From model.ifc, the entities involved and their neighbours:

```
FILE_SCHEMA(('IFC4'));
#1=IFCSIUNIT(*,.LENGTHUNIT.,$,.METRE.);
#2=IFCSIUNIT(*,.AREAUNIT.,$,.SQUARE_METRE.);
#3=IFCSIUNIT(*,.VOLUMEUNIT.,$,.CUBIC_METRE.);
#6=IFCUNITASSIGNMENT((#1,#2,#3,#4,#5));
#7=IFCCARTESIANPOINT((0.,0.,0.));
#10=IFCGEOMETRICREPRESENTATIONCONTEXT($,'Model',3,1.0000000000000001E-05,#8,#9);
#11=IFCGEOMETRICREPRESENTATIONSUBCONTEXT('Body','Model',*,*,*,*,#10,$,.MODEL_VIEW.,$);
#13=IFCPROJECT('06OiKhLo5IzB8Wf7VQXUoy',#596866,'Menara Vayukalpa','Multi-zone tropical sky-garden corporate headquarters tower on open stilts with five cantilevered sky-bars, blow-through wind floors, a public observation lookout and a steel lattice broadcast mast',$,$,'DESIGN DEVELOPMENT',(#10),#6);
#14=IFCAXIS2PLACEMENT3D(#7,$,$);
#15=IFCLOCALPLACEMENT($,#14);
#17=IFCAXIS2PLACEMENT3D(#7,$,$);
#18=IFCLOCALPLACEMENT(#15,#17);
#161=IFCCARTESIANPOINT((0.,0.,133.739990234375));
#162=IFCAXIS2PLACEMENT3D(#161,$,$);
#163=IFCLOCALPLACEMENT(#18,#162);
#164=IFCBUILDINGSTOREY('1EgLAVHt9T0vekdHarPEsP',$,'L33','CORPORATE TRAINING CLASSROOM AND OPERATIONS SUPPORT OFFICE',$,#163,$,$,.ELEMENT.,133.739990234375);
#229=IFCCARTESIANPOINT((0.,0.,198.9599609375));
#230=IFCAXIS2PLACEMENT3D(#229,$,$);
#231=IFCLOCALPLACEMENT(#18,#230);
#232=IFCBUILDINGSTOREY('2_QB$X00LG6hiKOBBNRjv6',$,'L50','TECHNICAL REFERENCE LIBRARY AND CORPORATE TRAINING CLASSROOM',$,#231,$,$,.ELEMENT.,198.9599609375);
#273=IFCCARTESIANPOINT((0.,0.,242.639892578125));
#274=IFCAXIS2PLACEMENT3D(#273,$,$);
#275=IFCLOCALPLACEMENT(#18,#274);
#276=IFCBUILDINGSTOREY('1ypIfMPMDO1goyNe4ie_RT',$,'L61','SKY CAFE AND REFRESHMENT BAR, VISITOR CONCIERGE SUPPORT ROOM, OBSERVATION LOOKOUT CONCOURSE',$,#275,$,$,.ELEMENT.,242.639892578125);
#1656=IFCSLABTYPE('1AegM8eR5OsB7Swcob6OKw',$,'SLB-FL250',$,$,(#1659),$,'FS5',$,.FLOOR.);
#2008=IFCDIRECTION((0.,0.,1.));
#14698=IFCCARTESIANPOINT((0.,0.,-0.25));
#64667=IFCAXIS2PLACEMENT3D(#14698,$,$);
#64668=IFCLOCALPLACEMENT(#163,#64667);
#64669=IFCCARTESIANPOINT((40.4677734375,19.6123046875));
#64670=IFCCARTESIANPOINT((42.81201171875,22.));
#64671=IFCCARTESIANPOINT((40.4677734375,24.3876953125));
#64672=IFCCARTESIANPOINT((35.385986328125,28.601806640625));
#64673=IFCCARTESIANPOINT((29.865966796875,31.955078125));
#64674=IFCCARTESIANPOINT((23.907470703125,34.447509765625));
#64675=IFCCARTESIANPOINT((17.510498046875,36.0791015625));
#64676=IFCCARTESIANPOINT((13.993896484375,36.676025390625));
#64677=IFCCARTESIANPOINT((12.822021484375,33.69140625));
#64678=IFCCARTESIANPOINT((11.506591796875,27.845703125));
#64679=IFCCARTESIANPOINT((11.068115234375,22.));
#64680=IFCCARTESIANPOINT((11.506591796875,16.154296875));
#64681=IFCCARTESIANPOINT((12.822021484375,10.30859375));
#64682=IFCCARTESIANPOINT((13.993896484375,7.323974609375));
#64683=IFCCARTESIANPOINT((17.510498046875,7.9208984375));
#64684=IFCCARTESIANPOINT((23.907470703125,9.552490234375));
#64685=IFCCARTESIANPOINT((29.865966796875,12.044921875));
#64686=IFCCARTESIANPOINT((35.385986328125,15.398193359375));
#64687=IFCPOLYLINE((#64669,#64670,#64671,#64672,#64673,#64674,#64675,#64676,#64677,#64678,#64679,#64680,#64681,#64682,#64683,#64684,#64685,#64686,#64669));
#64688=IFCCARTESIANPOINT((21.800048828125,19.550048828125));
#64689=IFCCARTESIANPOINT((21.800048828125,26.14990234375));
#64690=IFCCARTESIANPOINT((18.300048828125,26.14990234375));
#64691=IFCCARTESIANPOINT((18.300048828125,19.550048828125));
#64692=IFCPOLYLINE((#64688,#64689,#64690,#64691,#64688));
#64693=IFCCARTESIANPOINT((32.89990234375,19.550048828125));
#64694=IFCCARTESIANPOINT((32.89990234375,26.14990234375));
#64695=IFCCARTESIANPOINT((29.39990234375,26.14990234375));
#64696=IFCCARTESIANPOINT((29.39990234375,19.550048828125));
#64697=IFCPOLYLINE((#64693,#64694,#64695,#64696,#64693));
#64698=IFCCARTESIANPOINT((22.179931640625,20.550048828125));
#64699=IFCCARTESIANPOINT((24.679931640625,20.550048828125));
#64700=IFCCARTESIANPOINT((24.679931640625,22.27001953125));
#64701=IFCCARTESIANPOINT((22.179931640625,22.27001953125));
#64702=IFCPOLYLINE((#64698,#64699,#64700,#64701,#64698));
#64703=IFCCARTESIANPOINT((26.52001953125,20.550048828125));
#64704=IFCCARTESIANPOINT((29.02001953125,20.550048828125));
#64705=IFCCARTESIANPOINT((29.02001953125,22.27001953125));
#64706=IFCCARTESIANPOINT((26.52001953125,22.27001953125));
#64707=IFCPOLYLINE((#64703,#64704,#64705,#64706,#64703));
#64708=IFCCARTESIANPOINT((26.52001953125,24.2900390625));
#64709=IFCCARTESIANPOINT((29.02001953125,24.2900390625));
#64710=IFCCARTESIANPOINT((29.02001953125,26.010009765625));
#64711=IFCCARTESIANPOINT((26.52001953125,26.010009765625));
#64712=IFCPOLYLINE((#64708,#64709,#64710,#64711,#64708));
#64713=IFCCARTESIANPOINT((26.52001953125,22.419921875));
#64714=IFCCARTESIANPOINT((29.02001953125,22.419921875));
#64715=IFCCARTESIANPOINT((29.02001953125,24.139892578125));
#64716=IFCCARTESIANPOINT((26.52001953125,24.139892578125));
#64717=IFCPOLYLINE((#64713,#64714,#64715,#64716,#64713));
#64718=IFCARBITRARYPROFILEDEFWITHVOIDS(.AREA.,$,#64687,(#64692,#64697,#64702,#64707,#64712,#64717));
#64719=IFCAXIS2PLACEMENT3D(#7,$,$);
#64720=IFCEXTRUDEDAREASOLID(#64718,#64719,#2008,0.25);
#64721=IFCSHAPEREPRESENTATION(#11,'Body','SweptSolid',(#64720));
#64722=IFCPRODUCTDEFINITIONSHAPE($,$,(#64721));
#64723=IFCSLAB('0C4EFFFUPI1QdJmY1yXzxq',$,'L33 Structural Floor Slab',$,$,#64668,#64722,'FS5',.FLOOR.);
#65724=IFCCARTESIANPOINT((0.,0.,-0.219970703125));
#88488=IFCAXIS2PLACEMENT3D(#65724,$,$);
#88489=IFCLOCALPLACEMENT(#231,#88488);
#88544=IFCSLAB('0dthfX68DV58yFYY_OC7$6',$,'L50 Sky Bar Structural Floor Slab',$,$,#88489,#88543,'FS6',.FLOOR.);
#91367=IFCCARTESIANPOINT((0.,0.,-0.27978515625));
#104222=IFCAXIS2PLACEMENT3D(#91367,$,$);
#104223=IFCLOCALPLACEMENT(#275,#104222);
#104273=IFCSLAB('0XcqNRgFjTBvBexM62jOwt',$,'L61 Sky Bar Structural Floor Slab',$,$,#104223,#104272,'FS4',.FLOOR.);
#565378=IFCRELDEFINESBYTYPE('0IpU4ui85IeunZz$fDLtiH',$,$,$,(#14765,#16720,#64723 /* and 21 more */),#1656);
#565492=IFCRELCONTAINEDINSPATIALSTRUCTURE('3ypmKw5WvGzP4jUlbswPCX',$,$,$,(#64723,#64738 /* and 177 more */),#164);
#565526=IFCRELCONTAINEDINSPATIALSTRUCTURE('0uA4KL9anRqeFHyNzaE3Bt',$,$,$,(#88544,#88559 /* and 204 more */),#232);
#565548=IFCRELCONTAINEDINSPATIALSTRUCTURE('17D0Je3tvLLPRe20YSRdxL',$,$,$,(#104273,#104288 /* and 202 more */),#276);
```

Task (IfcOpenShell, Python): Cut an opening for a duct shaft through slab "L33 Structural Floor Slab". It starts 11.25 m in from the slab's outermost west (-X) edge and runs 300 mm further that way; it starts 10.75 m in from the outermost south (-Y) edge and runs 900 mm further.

```python
import numpy as np
import ifcopenshell
import ifcopenshell.api.feature
import ifcopenshell.api.geometry
import ifcopenshell.api.root
import ifcopenshell.geom
import ifcopenshell.util.placement
import ifcopenshell.util.representation
import ifcopenshell.util.shape
import ifcopenshell.util.unit

model = ifcopenshell.open("model.ifc")
unit_scale = ifcopenshell.util.unit.calculate_unit_scale(model)
settings = ifcopenshell.geom.settings()


def volume(element):
    """Net volume in cubic metres, openings subtracted."""
    shape = ifcopenshell.geom.create_shape(settings, element)
    return ifcopenshell.util.shape.get_volume(shape.geometry)


slab = model.by_guid("0C4EFFFUPI1QdJmY1yXzxq")
before = volume(slab)

# Extent in the slab's own axes, in metres. The edges named are its -X and -Y sides.
slab_shape = ifcopenshell.geom.create_shape(settings, slab)
vertices = ifcopenshell.util.shape.get_vertices(slab_shape.geometry)
x_min, y_min, bottom = vertices.min(axis=0)
top = vertices[:, 2].max()

opening = ifcopenshell.api.root.create_entity(model, ifc_class="IfcOpeningElement", name="Duct shaft opening", predefined_type="OPENING")
context = ifcopenshell.util.representation.get_context(model, "Model", "Body", "MODEL_VIEW")
width, depth = 0.3, 0.9
outline = [(0.0, 0.0), (width, 0.0), (width, depth), (0.0, depth), (0.0, 0.0)]
# Overshoot both faces by 50 mm so the cut is clean.
shape = ifcopenshell.api.geometry.add_slab_representation(
    model, context=context, depth=top - bottom + 0.1, polyline=outline
)
ifcopenshell.api.geometry.assign_representation(model, product=opening, representation=shape)

matrix = ifcopenshell.util.placement.get_local_placement(slab.ObjectPlacement)
matrix[:, 3] = matrix @ np.append(np.array([x_min + 11.25, y_min + 10.75, bottom - 0.05]) / unit_scale, 1.0)
ifcopenshell.api.geometry.edit_object_placement(model, product=opening, matrix=matrix, is_si=False)
ifcopenshell.api.feature.add_feature(model, feature=opening, element=slab)

after = volume(slab)

print(f"slab volume {before:.3f} -> {after:.3f} m3")

model.write("model_updated.ifc")
```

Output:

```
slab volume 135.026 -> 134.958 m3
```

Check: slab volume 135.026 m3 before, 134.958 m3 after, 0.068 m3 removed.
